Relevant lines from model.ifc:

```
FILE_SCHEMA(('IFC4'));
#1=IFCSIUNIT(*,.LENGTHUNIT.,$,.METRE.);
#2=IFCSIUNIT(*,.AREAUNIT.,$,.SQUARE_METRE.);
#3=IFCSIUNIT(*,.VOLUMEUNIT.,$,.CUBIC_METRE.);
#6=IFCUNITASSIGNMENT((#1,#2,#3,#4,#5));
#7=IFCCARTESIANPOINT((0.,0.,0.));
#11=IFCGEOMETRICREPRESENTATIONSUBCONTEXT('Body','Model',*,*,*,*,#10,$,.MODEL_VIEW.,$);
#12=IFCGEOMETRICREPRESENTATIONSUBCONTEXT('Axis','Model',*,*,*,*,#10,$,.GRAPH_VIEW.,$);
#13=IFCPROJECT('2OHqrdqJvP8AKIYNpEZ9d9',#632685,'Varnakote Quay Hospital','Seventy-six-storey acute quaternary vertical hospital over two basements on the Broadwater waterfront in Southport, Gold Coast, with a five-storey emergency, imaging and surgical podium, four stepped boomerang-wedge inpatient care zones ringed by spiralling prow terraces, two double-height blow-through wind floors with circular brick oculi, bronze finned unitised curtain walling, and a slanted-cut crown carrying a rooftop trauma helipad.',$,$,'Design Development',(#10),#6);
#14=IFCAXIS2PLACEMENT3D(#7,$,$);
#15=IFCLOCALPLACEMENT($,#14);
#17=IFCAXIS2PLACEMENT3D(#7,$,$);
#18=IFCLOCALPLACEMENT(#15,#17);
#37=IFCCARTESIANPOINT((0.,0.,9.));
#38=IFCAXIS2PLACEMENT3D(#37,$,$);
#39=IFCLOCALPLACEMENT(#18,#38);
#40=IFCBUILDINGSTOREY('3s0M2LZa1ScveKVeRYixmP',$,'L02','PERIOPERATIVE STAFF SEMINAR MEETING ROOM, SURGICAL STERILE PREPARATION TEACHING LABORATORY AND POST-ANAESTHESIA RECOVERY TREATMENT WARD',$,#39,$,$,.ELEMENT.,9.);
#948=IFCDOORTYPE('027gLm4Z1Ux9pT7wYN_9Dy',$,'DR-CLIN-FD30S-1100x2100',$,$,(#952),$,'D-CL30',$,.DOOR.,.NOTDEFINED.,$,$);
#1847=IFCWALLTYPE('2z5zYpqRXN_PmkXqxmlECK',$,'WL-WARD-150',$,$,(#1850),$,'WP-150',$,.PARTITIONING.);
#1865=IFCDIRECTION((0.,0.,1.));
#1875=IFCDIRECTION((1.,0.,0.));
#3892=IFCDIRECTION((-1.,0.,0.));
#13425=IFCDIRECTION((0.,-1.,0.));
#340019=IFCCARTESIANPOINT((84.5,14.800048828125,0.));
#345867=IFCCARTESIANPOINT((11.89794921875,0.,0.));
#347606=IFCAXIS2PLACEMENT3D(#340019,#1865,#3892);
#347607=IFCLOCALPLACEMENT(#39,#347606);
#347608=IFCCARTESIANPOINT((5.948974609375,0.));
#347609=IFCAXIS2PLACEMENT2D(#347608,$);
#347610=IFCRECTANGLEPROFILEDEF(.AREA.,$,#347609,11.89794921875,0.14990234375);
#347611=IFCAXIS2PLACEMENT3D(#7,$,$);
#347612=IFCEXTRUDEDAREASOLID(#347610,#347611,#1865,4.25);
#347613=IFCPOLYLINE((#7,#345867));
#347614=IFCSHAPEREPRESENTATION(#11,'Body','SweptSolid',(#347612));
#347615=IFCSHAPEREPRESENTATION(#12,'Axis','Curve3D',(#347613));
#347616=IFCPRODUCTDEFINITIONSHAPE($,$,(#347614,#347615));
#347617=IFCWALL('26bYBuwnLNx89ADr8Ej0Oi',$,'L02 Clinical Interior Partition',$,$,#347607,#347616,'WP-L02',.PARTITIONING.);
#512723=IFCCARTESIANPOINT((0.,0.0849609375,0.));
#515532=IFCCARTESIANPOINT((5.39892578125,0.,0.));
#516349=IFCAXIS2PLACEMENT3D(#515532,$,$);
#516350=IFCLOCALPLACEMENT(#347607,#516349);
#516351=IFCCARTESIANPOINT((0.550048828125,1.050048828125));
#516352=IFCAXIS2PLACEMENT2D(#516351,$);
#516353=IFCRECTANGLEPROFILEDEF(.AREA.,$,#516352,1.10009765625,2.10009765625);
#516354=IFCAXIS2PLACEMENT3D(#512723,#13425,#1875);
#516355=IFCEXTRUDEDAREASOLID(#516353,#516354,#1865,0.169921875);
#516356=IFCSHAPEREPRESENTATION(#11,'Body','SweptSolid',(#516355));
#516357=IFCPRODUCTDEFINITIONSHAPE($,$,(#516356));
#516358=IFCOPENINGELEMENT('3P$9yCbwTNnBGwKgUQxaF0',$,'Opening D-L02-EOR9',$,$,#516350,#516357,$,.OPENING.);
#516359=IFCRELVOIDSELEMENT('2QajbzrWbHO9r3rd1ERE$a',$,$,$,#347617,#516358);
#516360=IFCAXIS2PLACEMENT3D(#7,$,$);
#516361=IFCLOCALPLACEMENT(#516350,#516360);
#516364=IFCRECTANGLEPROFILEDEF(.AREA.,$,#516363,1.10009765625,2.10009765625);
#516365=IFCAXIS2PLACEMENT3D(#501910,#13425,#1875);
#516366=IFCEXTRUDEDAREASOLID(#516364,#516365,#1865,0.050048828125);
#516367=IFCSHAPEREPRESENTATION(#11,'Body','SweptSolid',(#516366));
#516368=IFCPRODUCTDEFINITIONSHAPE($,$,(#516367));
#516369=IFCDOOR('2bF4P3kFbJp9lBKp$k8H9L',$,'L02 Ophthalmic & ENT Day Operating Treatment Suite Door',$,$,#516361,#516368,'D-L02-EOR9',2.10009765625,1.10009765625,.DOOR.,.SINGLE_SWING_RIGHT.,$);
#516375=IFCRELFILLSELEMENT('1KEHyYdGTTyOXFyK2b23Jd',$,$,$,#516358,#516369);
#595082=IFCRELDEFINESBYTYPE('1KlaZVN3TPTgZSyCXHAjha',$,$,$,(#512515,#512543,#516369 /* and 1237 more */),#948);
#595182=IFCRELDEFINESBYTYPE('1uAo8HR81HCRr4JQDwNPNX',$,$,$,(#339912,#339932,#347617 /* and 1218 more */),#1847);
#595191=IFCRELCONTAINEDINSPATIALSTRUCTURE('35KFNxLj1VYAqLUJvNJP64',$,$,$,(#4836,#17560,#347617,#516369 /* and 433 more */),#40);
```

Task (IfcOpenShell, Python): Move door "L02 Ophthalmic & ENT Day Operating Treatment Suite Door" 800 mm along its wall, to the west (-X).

```python
import ifcopenshell
import ifcopenshell.api.geometry
import ifcopenshell.util.placement
import ifcopenshell.util.unit

model = ifcopenshell.open("model.ifc")
unit_scale = ifcopenshell.util.unit.calculate_unit_scale(model)

door = model.by_guid("2bF4P3kFbJp9lBKp$k8H9L")
opening = door.FillsVoids[0].RelatingOpeningElement
wall = opening.VoidsElements[0].RelatingBuildingElement

wall_matrix = ifcopenshell.util.placement.get_local_placement(wall.ObjectPlacement)
shift = wall_matrix[:3, 0] * 0.8 / unit_scale
before = ifcopenshell.util.placement.get_local_placement(door.ObjectPlacement)[:3, 3].copy()

# The door is placed relative to its opening, so it follows when the opening moves.
matrix = ifcopenshell.util.placement.get_local_placement(opening.ObjectPlacement)
matrix[:3, 3] += shift
ifcopenshell.api.geometry.edit_object_placement(
    model, product=opening, matrix=matrix, is_si=False, should_transform_children=True
)

after = ifcopenshell.util.placement.get_local_placement(door.ObjectPlacement)[:3, 3]
print("door moved by", (after - before).round(3) + 0.0)

model.write("model_rev.ifc")
```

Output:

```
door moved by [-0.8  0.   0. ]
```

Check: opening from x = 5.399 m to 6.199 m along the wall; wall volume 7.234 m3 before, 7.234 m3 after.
